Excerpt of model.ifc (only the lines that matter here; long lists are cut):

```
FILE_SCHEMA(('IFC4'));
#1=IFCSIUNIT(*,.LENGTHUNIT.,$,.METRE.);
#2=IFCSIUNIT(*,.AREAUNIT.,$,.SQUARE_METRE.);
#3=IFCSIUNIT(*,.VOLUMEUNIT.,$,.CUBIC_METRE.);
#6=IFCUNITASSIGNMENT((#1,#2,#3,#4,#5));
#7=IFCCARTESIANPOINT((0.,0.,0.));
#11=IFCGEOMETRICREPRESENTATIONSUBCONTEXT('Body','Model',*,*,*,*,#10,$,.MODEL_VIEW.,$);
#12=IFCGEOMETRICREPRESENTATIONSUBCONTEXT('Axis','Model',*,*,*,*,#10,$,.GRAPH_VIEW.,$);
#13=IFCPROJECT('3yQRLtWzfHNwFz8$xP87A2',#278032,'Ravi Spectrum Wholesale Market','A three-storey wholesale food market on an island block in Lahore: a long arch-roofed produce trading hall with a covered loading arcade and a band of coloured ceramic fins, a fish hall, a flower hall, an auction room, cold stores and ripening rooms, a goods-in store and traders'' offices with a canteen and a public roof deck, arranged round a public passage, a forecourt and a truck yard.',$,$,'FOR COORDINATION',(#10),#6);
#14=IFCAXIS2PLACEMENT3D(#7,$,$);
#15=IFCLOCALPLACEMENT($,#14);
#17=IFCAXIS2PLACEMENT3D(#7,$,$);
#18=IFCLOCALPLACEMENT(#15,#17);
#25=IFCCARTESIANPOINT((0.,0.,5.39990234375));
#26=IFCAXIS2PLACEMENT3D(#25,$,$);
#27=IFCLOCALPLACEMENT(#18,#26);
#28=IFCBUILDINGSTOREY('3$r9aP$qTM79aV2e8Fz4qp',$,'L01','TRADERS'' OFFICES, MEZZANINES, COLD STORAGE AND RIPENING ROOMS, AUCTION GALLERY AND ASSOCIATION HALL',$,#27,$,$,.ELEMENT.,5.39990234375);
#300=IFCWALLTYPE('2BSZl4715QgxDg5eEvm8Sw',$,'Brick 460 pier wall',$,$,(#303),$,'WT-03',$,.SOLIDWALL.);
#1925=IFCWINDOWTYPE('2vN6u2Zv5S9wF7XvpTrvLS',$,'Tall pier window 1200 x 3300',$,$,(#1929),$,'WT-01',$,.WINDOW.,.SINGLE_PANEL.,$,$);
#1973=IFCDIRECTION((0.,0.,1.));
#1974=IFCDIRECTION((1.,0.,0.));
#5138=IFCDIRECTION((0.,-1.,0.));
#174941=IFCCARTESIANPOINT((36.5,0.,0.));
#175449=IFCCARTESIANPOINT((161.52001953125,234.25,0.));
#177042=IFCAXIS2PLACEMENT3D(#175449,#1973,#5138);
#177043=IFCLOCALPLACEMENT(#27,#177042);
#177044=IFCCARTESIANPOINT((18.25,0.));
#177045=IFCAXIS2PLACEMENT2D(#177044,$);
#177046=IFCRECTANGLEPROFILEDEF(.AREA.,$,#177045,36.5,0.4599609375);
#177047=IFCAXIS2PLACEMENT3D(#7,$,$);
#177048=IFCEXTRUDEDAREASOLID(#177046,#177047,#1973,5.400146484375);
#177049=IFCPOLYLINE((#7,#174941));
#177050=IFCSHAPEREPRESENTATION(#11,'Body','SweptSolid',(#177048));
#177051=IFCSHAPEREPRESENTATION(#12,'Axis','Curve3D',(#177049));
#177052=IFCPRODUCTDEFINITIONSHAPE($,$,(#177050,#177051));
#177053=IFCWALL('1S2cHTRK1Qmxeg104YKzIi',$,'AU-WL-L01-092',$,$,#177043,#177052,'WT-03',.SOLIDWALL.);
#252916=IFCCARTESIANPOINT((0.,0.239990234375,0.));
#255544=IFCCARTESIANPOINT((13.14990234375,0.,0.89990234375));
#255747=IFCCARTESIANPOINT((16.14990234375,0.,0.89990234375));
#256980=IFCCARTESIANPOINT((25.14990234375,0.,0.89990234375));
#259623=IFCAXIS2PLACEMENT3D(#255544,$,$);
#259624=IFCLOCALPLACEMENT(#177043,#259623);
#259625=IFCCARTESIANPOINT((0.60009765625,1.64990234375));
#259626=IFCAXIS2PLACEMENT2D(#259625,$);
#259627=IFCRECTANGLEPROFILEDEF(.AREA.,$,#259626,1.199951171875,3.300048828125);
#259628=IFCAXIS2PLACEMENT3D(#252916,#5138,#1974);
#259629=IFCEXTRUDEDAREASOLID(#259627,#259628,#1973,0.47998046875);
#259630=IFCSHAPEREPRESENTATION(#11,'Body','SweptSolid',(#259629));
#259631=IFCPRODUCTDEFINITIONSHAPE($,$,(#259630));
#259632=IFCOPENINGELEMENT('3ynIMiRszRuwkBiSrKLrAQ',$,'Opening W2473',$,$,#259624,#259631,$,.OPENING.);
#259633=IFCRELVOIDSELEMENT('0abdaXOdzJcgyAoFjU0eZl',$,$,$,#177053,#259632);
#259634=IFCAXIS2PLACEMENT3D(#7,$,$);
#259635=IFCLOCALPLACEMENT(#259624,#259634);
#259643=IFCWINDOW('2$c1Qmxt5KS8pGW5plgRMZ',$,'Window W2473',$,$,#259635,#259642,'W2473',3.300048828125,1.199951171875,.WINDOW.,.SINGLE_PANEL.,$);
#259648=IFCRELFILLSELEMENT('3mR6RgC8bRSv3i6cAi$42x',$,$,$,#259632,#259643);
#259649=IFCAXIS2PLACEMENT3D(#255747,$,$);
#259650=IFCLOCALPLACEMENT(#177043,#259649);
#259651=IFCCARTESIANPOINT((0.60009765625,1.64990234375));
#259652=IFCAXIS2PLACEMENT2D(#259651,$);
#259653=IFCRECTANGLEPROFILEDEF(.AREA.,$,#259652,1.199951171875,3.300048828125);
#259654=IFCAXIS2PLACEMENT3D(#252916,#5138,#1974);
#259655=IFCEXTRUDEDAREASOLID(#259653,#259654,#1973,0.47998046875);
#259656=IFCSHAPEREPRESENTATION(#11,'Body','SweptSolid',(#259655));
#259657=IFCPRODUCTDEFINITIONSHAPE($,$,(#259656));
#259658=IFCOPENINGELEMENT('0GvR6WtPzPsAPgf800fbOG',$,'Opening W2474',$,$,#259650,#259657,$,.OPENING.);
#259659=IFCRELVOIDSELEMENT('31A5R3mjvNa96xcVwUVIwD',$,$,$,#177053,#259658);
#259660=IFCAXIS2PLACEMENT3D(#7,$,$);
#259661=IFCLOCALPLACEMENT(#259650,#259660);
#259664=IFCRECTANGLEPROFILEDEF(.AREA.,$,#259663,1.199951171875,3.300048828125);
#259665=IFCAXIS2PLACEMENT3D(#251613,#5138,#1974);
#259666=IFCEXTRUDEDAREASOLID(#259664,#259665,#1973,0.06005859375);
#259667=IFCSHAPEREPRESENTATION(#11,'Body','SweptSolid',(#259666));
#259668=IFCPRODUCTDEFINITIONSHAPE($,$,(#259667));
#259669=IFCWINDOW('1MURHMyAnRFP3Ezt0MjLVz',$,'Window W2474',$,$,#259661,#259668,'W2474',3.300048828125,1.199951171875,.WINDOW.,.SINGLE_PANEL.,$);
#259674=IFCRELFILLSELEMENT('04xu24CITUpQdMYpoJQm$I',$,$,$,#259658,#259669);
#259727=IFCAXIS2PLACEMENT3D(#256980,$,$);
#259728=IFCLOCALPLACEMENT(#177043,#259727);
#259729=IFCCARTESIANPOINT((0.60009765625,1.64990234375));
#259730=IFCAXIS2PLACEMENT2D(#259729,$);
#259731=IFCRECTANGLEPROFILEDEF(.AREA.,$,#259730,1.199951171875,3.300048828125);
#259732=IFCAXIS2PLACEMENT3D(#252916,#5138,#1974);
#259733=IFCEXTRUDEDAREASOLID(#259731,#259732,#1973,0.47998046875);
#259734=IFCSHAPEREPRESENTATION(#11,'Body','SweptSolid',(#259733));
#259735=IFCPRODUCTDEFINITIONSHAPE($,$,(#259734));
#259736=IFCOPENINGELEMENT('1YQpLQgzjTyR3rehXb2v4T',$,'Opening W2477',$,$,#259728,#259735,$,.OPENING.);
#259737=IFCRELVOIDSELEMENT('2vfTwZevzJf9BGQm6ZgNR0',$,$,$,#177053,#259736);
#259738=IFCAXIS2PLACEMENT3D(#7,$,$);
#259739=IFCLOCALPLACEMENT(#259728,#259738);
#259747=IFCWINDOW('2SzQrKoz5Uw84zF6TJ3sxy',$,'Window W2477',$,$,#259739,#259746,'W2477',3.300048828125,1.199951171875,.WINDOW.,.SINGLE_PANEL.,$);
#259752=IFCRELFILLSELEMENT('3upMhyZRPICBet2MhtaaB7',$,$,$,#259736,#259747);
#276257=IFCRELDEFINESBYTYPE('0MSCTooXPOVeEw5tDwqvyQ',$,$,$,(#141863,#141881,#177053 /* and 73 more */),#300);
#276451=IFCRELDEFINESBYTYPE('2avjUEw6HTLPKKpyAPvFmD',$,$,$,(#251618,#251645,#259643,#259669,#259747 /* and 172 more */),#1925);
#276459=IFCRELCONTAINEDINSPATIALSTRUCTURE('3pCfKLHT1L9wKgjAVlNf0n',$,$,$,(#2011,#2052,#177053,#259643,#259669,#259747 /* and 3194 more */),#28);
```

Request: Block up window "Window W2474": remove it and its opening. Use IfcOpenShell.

```python
import ifcopenshell
import ifcopenshell.api.feature
import ifcopenshell.api.root
import ifcopenshell.geom
import ifcopenshell.util.shape

model = ifcopenshell.open("model.ifc")
settings = ifcopenshell.geom.settings()


def volume(element):
    """Net volume in cubic metres, openings subtracted."""
    shape = ifcopenshell.geom.create_shape(settings, element)
    return ifcopenshell.util.shape.get_volume(shape.geometry)


window = model.by_id(259669)
opening = window.FillsVoids[0].RelatingOpeningElement
wall = opening.VoidsElements[0].RelatingBuildingElement
before = volume(wall)

ifcopenshell.api.root.remove_product(model, product=window)
ifcopenshell.api.feature.remove_feature(model, feature=opening)

after = volume(wall)

print(f"wall volume {before:.3f} -> {after:.3f} m3")

model.write("model_updated.ifc")
```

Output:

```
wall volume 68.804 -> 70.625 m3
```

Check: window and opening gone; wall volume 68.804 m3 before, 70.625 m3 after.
